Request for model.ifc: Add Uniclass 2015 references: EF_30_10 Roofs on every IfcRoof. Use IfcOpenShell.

First a look at what the model holds.

```python
import ifcopenshell

model = ifcopenshell.open("model.ifc")
print(model.schema)
print("classifications:", [c.Name for c in model.by_type("IfcClassification")])
for ifc_class in ("IfcDoor", "IfcRoof", "IfcStair", "IfcWall", "IfcWindow"):
    print(ifc_class, len(model.by_type(ifc_class)))
```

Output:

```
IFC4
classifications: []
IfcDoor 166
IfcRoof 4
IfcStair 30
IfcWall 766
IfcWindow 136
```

```python
import ifcopenshell
import ifcopenshell.api.classification

model = ifcopenshell.open("model.ifc")

system = ifcopenshell.api.classification.add_classification(model, classification="Uniclass 2015")

codes = {
    "IfcRoof": ("EF_30_10", "Roofs"),
}
for ifc_class, (code, name) in codes.items():
    products = model.by_type(ifc_class)
    ifcopenshell.api.classification.add_reference(
        model, products=products, classification=system, identification=code, name=name
    )
    print(code, len(products))

model.write("model_rev.ifc")
```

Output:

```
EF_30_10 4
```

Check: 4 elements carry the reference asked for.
